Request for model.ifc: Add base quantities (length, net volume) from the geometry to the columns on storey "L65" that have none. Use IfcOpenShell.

First a look at what the model holds.

```python
import ifcopenshell
import ifcopenshell.util.element
import ifcopenshell.util.unit

model = ifcopenshell.open("model.ifc")
print(model.schema)
for unit_type in ("LENGTHUNIT", "AREAUNIT", "VOLUMEUNIT"):
    print(unit_type, ifcopenshell.util.unit.calculate_unit_scale(model, unit_type))
storey = next(s for s in model.by_type("IfcBuildingStorey") if s.Name == "L65")
columns = [e for e in ifcopenshell.util.element.get_decomposition(storey) if e.is_a("IfcColumn")]
for e in sorted(columns, key=lambda e: e.id()):
    print(e.id(), e.is_a(), e.Name, list(ifcopenshell.util.element.get_psets(e, qtos_only=True)), sep=" | ")
```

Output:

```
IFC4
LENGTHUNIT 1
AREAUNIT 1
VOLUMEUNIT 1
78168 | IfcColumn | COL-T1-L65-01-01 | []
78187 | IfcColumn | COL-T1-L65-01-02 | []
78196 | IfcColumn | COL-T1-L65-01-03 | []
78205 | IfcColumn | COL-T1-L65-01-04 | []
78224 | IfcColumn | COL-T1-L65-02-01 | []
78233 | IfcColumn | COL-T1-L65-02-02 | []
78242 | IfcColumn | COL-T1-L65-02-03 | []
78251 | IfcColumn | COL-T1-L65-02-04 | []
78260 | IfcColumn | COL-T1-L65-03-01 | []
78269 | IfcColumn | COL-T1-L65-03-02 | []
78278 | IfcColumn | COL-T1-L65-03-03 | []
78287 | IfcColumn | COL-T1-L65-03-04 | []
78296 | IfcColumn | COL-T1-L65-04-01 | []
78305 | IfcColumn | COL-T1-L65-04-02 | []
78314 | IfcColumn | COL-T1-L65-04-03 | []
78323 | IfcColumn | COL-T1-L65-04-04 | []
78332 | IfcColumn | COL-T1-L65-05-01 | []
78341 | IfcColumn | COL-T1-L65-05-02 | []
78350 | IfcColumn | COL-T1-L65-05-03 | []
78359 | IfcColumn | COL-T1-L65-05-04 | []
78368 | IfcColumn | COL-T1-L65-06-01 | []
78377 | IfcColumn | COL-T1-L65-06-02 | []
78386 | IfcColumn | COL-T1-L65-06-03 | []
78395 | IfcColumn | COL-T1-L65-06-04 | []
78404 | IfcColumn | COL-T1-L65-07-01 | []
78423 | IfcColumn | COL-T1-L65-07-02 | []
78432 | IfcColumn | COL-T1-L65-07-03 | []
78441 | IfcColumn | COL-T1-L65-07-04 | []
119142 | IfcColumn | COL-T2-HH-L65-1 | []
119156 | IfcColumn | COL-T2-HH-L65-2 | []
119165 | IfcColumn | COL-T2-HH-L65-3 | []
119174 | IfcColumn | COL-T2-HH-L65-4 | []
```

```python
import ifcopenshell
import ifcopenshell.api.pset
import ifcopenshell.geom
import ifcopenshell.util.element
import ifcopenshell.util.shape
import ifcopenshell.util.unit

model = ifcopenshell.open("model.ifc")
unit_scale = ifcopenshell.util.unit.calculate_unit_scale(model)
volume_scale = ifcopenshell.util.unit.calculate_unit_scale(model, "VOLUMEUNIT")
settings = ifcopenshell.geom.settings()

storey = next(s for s in model.by_type("IfcBuildingStorey") if s.Name == "L65")
columns = [e for e in ifcopenshell.util.element.get_decomposition(storey) if e.is_a("IfcColumn")]

for e in sorted(columns, key=lambda e: e.id()):
    if ifcopenshell.util.element.get_psets(e, qtos_only=True, should_inherit=False):
        continue
    # Geometry comes back in metres, in the element's own axes.
    shape = ifcopenshell.geom.create_shape(settings, e)
    values = {
        "Length": ifcopenshell.util.shape.get_z(shape.geometry) / unit_scale,
        "NetVolume": ifcopenshell.util.shape.get_volume(shape.geometry) / volume_scale,
    }
    qto = ifcopenshell.api.pset.add_qto(model, product=e, name="Qto_ColumnBaseQuantities")
    ifcopenshell.api.pset.edit_qto(model, qto=qto, properties=values)
    print(e.id(), {k: round(v, 3) for k, v in values.items()})

model.write("model-out.ifc")
```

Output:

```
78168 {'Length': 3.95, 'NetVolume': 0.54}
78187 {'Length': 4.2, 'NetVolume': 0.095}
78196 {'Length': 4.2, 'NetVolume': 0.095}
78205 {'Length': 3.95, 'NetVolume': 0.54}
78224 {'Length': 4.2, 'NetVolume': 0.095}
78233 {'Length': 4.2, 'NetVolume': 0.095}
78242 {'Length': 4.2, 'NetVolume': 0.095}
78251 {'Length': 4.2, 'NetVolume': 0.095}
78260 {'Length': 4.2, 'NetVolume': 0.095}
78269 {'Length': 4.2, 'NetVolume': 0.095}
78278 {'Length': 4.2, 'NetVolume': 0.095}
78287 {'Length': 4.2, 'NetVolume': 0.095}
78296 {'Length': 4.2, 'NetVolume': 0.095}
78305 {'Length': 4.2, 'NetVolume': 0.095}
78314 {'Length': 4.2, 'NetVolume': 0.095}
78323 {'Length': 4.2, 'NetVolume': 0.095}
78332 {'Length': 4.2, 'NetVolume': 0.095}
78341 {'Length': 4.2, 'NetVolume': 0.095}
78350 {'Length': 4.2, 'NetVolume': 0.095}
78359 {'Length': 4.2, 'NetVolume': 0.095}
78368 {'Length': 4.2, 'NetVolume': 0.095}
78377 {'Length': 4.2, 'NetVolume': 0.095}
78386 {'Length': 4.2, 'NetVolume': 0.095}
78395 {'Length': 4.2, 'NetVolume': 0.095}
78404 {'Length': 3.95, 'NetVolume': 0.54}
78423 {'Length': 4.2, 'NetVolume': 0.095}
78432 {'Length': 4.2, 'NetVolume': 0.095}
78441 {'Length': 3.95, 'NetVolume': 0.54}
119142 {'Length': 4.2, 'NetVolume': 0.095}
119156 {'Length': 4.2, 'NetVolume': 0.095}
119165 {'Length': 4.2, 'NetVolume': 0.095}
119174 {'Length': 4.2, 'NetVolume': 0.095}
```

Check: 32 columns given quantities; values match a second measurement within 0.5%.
